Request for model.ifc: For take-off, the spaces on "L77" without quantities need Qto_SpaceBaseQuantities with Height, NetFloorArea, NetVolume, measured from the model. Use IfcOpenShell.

First a look at what the model holds.

```python
import ifcopenshell
import ifcopenshell.util.element
import ifcopenshell.util.unit

model = ifcopenshell.open("model.ifc")
print(model.schema)
for unit_type in ("LENGTHUNIT", "AREAUNIT", "VOLUMEUNIT"):
    print(unit_type, ifcopenshell.util.unit.calculate_unit_scale(model, unit_type))
storey = next(s for s in model.by_type("IfcBuildingStorey") if s.Name == "L77")
spaces = [e for e in ifcopenshell.util.element.get_decomposition(storey) if e.is_a("IfcSpace")]
for e in sorted(spaces, key=lambda e: e.id()):
    print(e.id(), e.is_a(), e.Name, list(ifcopenshell.util.element.get_psets(e, qtos_only=True)), sep=" | ")
```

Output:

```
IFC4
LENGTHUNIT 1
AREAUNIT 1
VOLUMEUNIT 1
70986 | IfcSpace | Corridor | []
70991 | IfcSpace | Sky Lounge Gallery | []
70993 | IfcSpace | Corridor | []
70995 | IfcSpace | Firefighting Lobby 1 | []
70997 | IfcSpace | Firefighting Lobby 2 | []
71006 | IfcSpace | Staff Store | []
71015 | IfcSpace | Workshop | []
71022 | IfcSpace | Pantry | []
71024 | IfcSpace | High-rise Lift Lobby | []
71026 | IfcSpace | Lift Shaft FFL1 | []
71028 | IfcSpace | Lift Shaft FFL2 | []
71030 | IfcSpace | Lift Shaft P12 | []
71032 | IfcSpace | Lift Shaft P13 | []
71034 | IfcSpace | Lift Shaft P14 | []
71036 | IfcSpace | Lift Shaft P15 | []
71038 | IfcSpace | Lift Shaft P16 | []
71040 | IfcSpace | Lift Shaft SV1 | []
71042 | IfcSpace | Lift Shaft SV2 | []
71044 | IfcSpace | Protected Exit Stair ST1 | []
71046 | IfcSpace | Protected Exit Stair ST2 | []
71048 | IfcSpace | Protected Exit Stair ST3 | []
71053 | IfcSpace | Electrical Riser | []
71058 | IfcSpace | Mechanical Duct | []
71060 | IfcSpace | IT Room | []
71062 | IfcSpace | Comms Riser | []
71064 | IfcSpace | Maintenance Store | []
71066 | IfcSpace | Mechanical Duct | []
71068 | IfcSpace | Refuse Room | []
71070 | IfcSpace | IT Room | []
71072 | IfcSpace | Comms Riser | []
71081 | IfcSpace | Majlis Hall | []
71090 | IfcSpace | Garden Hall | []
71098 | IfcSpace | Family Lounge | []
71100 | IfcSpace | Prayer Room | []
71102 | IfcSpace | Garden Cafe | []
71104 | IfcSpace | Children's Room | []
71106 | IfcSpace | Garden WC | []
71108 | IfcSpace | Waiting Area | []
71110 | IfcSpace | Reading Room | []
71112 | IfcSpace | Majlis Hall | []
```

```python
import ifcopenshell
import ifcopenshell.api.pset
import ifcopenshell.geom
import ifcopenshell.util.element
import ifcopenshell.util.shape
import ifcopenshell.util.unit

model = ifcopenshell.open("model.ifc")
unit_scale = ifcopenshell.util.unit.calculate_unit_scale(model)
area_scale = ifcopenshell.util.unit.calculate_unit_scale(model, "AREAUNIT")
volume_scale = ifcopenshell.util.unit.calculate_unit_scale(model, "VOLUMEUNIT")
settings = ifcopenshell.geom.settings()

storey = next(s for s in model.by_type("IfcBuildingStorey") if s.Name == "L77")
spaces = [e for e in ifcopenshell.util.element.get_decomposition(storey) if e.is_a("IfcSpace")]

for e in sorted(spaces, key=lambda e: e.id()):
    if ifcopenshell.util.element.get_psets(e, qtos_only=True, should_inherit=False):
        continue
    # Geometry comes back in metres, in the element's own axes.
    shape = ifcopenshell.geom.create_shape(settings, e)
    values = {
        "Height": ifcopenshell.util.shape.get_z(shape.geometry) / unit_scale,
        "NetFloorArea": ifcopenshell.util.shape.get_footprint_area(shape.geometry) / area_scale,
        "NetVolume": ifcopenshell.util.shape.get_volume(shape.geometry) / volume_scale,
    }
    qto = ifcopenshell.api.pset.add_qto(model, product=e, name="Qto_SpaceBaseQuantities")
    ifcopenshell.api.pset.edit_qto(model, qto=qto, properties=values)
    print(e.id(), {k: round(v, 3) for k, v in values.items()})

model.write("model_edited.ifc")
```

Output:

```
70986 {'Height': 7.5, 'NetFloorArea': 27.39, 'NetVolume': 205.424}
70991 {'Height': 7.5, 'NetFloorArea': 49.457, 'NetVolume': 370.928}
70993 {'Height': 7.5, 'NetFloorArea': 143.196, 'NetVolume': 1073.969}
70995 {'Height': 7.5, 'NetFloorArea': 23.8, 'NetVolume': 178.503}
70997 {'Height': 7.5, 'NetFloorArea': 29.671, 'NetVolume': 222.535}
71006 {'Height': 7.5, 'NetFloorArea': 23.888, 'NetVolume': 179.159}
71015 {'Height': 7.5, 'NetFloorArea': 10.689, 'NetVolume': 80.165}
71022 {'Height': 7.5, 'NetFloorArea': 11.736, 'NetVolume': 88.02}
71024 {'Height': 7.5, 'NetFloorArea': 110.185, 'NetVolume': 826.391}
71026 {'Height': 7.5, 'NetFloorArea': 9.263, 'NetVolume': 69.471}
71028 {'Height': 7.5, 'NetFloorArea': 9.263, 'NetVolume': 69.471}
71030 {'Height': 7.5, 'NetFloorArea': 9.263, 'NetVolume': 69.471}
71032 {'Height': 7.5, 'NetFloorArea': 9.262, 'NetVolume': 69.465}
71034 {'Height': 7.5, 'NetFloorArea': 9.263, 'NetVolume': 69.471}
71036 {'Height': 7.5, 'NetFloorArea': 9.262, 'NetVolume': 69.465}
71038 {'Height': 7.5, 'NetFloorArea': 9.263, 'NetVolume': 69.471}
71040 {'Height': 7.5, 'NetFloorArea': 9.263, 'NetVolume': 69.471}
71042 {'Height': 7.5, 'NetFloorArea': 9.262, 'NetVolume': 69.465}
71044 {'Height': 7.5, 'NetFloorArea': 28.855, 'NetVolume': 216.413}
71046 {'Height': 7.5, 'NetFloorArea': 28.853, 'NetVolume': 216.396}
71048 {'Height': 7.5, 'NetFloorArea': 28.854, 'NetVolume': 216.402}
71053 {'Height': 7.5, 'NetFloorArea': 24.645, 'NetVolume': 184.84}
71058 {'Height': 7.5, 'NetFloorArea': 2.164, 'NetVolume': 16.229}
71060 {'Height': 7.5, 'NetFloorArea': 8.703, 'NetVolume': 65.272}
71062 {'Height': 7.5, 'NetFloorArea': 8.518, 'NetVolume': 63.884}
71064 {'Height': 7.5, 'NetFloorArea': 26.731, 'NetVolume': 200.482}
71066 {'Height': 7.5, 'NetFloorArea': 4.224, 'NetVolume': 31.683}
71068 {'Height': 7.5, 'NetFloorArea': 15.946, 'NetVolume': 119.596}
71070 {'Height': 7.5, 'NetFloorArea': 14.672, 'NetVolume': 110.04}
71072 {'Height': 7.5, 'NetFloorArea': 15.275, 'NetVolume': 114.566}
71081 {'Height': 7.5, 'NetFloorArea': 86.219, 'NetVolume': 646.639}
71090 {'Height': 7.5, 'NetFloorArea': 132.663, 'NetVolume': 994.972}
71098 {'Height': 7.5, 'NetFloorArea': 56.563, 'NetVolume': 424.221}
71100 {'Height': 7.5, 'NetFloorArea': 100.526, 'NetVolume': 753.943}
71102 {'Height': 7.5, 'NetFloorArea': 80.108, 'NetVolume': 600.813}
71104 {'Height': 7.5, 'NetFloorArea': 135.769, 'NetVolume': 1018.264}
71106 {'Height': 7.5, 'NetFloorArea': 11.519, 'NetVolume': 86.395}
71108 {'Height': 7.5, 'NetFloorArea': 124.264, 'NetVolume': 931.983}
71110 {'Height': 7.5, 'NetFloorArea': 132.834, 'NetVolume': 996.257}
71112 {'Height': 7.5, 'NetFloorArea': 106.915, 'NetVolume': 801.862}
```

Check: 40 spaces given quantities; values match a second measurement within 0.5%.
